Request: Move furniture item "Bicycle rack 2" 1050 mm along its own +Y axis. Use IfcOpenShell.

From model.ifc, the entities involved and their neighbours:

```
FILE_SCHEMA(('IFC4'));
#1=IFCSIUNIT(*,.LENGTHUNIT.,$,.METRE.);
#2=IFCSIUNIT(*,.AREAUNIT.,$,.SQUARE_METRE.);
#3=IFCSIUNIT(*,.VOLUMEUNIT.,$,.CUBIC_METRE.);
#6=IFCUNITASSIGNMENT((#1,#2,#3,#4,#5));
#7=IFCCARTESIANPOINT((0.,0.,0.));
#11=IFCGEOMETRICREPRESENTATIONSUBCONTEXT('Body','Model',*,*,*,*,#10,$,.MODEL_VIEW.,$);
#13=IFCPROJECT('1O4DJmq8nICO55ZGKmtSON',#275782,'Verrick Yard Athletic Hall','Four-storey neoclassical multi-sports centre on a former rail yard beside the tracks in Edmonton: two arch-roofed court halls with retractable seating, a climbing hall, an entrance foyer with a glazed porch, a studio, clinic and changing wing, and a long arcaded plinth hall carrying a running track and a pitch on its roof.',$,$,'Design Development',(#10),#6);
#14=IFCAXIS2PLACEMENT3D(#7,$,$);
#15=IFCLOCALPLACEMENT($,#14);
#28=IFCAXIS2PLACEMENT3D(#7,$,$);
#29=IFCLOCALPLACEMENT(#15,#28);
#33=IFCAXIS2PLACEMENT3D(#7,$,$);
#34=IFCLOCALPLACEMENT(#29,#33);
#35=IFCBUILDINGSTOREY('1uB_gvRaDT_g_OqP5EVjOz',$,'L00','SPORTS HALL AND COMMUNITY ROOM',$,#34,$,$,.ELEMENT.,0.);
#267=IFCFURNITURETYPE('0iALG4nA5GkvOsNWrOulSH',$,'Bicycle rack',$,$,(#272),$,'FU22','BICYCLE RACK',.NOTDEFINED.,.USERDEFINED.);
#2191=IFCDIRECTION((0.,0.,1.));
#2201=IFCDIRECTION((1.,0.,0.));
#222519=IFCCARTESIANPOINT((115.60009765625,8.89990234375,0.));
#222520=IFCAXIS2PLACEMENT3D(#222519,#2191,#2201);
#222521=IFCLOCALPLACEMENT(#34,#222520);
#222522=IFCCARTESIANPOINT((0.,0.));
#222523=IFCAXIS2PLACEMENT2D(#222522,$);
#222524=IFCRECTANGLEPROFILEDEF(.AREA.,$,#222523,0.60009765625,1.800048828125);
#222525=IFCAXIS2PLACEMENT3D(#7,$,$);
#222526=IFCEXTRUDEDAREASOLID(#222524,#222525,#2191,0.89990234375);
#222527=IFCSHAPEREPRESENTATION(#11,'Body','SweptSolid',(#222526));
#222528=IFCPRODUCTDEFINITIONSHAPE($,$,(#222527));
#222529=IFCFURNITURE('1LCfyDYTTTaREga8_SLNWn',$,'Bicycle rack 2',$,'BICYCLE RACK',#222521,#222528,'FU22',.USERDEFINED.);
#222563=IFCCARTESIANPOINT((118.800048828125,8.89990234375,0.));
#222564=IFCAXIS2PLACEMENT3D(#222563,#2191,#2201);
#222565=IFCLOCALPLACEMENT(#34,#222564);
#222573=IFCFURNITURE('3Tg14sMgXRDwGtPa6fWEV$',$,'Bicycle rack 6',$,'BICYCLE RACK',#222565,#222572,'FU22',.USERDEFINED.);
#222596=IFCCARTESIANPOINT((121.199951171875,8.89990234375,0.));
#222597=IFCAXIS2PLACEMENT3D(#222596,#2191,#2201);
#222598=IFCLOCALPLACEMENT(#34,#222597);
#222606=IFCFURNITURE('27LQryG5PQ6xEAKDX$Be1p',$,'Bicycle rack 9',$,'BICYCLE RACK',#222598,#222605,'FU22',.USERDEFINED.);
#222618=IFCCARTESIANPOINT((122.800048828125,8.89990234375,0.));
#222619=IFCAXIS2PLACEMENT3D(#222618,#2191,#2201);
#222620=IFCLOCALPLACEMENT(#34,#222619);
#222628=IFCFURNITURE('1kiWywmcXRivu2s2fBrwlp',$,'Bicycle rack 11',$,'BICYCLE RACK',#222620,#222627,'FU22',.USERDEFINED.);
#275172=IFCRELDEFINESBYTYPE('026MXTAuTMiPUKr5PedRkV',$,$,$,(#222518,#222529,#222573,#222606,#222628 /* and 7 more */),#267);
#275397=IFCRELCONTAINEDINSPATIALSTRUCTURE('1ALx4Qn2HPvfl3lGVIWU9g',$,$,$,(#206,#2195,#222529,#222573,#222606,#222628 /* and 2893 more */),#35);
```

```python
import ifcopenshell
import ifcopenshell.api.geometry
import ifcopenshell.util.placement
import ifcopenshell.util.unit

model = ifcopenshell.open("model.ifc")
unit_scale = ifcopenshell.util.unit.calculate_unit_scale(model)

item = model.by_guid("1LCfyDYTTTaREga8_SLNWn")
matrix = ifcopenshell.util.placement.get_local_placement(item.ObjectPlacement)
matrix[:3, 3] += matrix[:3, 1] * 1.05 / unit_scale
ifcopenshell.api.geometry.edit_object_placement(model, product=item, matrix=matrix, is_si=False)

print(ifcopenshell.util.placement.get_local_placement(item.ObjectPlacement).round(3) + 0.0)

model.write("model_rev.ifc")
```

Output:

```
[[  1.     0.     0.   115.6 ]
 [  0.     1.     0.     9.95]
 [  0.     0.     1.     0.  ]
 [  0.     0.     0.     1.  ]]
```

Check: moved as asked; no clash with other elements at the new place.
